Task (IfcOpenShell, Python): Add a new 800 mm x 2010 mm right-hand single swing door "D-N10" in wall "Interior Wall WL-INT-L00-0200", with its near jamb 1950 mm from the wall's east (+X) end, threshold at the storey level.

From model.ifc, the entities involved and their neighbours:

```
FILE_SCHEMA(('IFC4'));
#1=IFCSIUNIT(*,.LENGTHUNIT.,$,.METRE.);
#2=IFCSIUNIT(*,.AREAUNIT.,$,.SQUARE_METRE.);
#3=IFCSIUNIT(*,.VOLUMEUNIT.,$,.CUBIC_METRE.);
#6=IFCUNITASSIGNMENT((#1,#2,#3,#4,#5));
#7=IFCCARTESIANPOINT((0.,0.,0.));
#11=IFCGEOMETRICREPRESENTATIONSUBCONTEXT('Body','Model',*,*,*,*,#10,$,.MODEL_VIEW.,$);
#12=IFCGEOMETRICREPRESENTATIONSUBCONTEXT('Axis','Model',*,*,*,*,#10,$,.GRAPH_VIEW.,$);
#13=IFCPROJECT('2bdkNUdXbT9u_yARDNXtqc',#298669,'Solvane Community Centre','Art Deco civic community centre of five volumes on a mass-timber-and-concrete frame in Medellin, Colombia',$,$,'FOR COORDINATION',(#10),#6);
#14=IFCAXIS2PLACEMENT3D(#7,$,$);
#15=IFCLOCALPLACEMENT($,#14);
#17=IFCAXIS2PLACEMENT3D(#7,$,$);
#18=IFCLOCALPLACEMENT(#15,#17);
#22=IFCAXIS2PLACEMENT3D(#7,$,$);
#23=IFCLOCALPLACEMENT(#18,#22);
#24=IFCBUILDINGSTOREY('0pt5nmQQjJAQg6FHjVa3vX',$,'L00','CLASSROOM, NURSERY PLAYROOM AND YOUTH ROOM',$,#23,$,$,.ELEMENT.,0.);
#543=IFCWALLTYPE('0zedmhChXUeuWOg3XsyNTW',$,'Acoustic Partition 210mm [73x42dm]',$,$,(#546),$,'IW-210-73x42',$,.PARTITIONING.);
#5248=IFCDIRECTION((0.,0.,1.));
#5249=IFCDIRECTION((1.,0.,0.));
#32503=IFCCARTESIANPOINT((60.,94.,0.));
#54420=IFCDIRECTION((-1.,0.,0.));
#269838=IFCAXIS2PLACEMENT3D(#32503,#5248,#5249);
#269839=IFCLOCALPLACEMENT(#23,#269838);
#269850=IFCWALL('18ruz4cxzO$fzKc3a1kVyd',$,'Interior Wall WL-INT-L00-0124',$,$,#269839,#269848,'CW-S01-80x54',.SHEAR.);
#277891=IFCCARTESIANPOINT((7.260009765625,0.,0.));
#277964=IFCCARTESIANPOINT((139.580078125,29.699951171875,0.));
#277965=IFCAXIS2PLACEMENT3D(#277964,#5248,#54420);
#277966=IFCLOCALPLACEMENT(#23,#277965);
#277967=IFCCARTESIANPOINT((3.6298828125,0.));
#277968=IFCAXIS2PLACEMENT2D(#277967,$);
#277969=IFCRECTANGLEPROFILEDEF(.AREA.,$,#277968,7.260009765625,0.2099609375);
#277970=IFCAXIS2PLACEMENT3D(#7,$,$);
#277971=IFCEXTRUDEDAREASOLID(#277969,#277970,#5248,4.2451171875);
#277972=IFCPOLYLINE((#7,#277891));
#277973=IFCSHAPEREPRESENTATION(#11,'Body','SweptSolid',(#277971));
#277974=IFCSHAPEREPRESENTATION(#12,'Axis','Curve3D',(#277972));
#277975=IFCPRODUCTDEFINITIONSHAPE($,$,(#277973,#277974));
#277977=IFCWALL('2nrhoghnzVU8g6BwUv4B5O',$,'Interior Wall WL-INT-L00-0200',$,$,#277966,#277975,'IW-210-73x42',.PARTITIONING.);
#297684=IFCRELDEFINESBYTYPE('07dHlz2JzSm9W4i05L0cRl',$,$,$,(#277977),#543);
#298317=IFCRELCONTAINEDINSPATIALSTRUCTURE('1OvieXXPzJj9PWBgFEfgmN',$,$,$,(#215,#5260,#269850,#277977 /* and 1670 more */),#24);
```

```python
import numpy as np
import ifcopenshell
import ifcopenshell.api.feature
import ifcopenshell.api.geometry
import ifcopenshell.api.root
import ifcopenshell.api.spatial
import ifcopenshell.geom
import ifcopenshell.util.element
import ifcopenshell.util.placement
import ifcopenshell.util.representation
import ifcopenshell.util.shape
import ifcopenshell.util.unit

model = ifcopenshell.open("model.ifc")
unit_scale = ifcopenshell.util.unit.calculate_unit_scale(model)
settings = ifcopenshell.geom.settings()


def volume(element):
    """Net volume in cubic metres, openings subtracted."""
    shape = ifcopenshell.geom.create_shape(settings, element)
    return ifcopenshell.util.shape.get_volume(shape.geometry)


wall = model.by_guid("2nrhoghnzVU8g6BwUv4B5O")
storey = ifcopenshell.util.element.get_container(wall, ifc_class="IfcBuildingStorey")
context = ifcopenshell.util.representation.get_context(model, "Model", "Body", "MODEL_VIEW")
before = volume(wall)

width, height, from_end, sill = 0.8, 2.01, 1.95, 0.0  # metres

# The wall runs along its own X axis, and the end named is its -X end.
wall_shape = ifcopenshell.geom.create_shape(settings, wall)
x, y, z = ifcopenshell.util.shape.get_vertices(wall_shape.geometry).T
start = x.min() + from_end
face, thickness = float(y.min()), float(y.max() - y.min())
wall_matrix = ifcopenshell.util.placement.get_local_placement(wall.ObjectPlacement)
level = ifcopenshell.util.placement.get_local_placement(storey.ObjectPlacement)[2, 3]


def in_wall(x, y):
    """Placement at x, y metres in the wall's axes, at sill height."""
    matrix = wall_matrix.copy()
    matrix[:, 3] = wall_matrix @ np.array([x / unit_scale, y / unit_scale, 0.0, 1.0])
    matrix[2, 3] = level + sill / unit_scale
    return matrix


# Opening: a box that overshoots both wall faces by 50 mm.
opening = ifcopenshell.api.root.create_entity(model, ifc_class="IfcOpeningElement", predefined_type="OPENING")
box = ifcopenshell.api.geometry.add_wall_representation(
    model, context=context, length=width, height=height, thickness=thickness + 0.1
)
ifcopenshell.api.geometry.assign_representation(model, product=opening, representation=box)
ifcopenshell.api.geometry.edit_object_placement(model, product=opening, matrix=in_wall(start, face - 0.05), is_si=False)
ifcopenshell.api.feature.add_feature(model, feature=opening, element=wall)

door = ifcopenshell.api.root.create_entity(model, ifc_class="IfcDoor", name="D-N10", predefined_type="DOOR")
door.OverallWidth, door.OverallHeight = width / unit_scale, height / unit_scale
door.OperationType = "SINGLE_SWING_RIGHT"
body = ifcopenshell.api.geometry.add_door_representation(
    model,
    context=context,
    overall_width=door.OverallWidth,
    overall_height=door.OverallHeight,
    operation_type="SINGLE_SWING_RIGHT",
    lining_properties={"LiningDepth": thickness / unit_scale, "ThresholdDepth": thickness / unit_scale},
)
ifcopenshell.api.geometry.assign_representation(model, product=door, representation=body)
ifcopenshell.api.spatial.assign_container(model, products=[door], relating_structure=storey)
ifcopenshell.api.feature.add_filling(model, opening=opening, element=door)

# The lining spans the wall, so the door starts at the wall face.
ifcopenshell.api.geometry.edit_object_placement(model, product=door, matrix=in_wall(start, face), is_si=False)

after = volume(wall)

print(f"wall volume {before:.3f} -> {after:.3f} m3")

model.write("model_updated.ifc")
```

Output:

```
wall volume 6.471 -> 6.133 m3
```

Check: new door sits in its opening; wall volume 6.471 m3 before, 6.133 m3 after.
